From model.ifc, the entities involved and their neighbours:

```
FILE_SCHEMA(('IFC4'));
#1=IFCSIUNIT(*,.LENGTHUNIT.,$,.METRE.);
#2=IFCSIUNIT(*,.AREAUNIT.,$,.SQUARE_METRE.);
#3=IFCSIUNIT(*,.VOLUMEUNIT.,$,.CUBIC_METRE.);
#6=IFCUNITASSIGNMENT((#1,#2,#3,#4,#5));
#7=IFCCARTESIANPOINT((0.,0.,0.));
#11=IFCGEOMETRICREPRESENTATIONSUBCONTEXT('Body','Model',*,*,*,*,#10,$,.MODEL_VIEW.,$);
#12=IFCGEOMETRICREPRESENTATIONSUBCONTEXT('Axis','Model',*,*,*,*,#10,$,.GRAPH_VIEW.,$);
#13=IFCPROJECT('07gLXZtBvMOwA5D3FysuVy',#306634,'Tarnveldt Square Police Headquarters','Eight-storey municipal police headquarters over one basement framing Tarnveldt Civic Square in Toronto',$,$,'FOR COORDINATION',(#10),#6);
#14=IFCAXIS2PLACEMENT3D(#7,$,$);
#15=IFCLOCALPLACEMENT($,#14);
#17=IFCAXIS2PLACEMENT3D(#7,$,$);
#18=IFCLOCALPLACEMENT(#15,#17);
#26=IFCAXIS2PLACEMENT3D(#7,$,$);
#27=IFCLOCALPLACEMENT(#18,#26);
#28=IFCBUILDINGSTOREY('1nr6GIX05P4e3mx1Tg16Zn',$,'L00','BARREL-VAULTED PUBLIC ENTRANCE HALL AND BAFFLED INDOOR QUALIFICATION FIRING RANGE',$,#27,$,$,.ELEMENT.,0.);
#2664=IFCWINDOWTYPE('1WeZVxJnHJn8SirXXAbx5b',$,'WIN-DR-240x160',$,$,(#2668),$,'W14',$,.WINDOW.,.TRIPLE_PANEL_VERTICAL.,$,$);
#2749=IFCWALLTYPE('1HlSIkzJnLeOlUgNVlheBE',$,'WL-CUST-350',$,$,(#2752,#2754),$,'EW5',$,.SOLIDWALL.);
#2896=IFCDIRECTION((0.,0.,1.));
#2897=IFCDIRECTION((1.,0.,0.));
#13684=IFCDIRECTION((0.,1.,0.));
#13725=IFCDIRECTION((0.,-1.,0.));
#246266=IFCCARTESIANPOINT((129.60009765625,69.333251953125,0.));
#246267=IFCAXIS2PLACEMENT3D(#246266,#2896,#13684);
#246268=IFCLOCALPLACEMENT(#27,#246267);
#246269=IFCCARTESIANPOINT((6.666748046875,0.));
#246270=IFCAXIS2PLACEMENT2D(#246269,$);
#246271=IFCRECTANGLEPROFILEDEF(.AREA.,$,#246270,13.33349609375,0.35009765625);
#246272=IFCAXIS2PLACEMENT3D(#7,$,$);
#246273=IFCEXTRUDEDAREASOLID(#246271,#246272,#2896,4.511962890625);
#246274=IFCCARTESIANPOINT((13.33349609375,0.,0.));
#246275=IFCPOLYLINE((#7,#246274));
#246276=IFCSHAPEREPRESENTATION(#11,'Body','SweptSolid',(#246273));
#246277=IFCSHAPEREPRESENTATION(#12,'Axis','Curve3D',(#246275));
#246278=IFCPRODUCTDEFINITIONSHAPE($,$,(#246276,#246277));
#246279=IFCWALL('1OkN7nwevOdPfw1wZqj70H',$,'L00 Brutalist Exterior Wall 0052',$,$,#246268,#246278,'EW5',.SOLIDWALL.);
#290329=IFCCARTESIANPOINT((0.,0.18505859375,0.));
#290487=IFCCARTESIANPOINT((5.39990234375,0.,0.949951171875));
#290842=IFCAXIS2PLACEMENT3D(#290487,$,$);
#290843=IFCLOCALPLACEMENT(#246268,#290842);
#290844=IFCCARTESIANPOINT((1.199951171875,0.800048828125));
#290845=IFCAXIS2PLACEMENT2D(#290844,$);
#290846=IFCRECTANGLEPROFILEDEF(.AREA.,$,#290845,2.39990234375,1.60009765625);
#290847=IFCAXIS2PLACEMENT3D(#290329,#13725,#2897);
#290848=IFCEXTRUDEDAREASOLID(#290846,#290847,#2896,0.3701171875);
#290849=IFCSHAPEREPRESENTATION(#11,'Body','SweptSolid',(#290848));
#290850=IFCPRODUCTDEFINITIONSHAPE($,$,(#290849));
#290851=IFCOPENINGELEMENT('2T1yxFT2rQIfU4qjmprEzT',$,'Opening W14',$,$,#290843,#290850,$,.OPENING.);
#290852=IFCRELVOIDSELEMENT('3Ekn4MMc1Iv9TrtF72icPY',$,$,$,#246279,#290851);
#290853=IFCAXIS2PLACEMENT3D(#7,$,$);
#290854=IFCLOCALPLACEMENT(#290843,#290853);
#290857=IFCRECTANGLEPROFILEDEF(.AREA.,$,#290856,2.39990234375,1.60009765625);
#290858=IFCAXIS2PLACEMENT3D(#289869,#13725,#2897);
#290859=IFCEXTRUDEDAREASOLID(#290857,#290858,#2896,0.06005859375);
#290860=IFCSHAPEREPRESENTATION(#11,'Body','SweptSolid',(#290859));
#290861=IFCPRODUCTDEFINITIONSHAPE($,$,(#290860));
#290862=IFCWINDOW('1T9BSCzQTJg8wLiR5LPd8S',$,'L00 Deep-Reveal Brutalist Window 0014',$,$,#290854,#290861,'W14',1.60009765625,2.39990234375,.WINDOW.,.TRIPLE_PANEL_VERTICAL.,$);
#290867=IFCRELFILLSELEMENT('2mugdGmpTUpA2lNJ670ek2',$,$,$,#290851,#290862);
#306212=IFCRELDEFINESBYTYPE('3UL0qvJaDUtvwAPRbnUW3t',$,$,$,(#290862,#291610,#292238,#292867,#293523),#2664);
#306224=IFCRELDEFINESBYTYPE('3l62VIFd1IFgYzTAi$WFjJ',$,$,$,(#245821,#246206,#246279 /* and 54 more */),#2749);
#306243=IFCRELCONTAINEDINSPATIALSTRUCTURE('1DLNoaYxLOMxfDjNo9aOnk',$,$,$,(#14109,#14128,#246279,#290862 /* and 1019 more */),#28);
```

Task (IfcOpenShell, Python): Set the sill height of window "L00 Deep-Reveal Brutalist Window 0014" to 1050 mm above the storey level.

```python
import numpy as np
import ifcopenshell
import ifcopenshell.api.geometry
import ifcopenshell.geom
import ifcopenshell.util.element
import ifcopenshell.util.placement
import ifcopenshell.util.shape
import ifcopenshell.util.unit

model = ifcopenshell.open("model.ifc")
unit_scale = ifcopenshell.util.unit.calculate_unit_scale(model)

window = model.by_guid("1T9BSCzQTJg8wLiR5LPd8S")
opening = window.FillsVoids[0].RelatingOpeningElement
storey = ifcopenshell.util.element.get_container(window, ifc_class="IfcBuildingStorey")
level = ifcopenshell.util.placement.get_local_placement(storey.ObjectPlacement)[2, 3]

# The opening's origin need not be at the sill, so measure its lowest point.
shape = ifcopenshell.geom.create_shape(ifcopenshell.geom.settings(), opening)
bottom = ifcopenshell.util.shape.get_shape_bottom_elevation(shape, shape.geometry) / unit_scale
dz = level + 1.05 / unit_scale - bottom

shift = np.array([0.0, 0.0, dz])
# The window is placed relative to its opening, so it follows when the opening moves.
matrix = ifcopenshell.util.placement.get_local_placement(opening.ObjectPlacement)
matrix[:3, 3] += shift
ifcopenshell.api.geometry.edit_object_placement(
    model, product=opening, matrix=matrix, is_si=False, should_transform_children=True
)

print(f"moved by {dz * unit_scale:+.3f} m")

model.write("model_updated.ifc")
```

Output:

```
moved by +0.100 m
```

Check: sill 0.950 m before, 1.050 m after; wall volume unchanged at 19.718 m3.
